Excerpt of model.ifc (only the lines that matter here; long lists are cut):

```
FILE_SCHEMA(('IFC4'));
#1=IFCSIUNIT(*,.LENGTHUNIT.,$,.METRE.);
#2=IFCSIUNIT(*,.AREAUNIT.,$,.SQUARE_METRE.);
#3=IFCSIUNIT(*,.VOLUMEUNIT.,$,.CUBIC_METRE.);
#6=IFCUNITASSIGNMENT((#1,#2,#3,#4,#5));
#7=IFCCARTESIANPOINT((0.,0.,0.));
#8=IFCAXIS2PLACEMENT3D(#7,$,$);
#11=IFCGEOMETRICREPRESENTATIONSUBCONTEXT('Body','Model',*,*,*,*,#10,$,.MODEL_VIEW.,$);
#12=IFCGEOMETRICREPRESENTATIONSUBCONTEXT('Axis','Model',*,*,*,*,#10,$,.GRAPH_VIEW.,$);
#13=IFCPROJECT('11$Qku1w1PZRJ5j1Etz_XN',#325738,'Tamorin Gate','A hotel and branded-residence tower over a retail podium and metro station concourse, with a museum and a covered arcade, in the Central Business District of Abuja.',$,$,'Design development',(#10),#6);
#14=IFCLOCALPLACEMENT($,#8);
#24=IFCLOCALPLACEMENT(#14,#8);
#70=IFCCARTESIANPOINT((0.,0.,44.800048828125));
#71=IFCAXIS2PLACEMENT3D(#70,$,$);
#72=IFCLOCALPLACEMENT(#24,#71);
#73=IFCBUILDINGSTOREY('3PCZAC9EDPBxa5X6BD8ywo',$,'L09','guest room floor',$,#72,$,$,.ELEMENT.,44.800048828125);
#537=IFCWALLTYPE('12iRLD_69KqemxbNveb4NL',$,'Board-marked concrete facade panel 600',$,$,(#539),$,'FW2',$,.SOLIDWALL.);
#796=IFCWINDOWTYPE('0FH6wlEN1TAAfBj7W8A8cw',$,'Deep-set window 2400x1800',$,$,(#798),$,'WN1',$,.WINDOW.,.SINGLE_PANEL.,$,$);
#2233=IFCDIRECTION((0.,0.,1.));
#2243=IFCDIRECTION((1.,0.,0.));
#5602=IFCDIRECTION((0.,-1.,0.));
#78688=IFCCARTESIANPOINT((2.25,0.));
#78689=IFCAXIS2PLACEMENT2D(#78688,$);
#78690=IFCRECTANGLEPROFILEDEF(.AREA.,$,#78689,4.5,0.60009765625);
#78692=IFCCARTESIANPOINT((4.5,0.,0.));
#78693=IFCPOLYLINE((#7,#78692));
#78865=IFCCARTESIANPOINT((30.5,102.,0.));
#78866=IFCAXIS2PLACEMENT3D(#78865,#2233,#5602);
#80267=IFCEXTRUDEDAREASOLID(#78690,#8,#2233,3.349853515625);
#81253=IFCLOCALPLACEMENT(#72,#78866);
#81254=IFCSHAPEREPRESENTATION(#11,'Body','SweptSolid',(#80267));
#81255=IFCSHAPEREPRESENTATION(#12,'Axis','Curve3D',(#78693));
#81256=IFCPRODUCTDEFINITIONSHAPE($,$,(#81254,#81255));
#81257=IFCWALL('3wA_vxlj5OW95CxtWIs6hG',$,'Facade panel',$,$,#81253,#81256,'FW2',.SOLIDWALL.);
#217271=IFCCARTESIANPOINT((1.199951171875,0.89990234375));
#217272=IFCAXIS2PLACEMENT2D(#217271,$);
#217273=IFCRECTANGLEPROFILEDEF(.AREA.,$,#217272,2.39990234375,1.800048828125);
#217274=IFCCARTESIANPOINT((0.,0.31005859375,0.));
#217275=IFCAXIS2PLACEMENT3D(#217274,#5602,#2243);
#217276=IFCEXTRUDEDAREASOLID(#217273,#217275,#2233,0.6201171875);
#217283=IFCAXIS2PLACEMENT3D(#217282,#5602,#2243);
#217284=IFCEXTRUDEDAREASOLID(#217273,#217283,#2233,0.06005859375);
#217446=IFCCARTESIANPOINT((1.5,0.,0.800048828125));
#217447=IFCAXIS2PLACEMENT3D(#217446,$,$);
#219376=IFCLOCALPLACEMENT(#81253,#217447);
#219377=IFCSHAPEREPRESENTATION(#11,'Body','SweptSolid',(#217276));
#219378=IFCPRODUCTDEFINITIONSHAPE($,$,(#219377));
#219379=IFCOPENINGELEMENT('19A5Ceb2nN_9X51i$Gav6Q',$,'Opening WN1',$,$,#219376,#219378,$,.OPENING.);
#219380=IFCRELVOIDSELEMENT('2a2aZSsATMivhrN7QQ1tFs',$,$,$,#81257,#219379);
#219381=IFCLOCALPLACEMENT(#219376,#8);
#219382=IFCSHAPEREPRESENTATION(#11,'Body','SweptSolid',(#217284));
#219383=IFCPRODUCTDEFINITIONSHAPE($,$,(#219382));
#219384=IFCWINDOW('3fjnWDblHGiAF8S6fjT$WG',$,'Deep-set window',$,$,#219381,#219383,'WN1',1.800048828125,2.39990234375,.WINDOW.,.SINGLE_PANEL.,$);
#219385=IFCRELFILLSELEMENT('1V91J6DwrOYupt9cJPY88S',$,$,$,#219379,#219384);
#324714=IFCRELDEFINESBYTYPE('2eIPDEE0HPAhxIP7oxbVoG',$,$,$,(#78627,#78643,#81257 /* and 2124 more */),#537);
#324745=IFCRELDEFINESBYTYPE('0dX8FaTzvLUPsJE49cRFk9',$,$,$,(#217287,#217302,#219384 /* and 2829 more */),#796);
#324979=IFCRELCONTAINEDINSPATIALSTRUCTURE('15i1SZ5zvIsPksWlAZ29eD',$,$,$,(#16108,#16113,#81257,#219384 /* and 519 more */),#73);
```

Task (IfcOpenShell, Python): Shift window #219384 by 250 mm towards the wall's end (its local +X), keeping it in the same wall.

```python
import ifcopenshell
import ifcopenshell.api.geometry
import ifcopenshell.util.placement
import ifcopenshell.util.unit

model = ifcopenshell.open("model.ifc")
unit_scale = ifcopenshell.util.unit.calculate_unit_scale(model)

window = model.by_guid("3fjnWDblHGiAF8S6fjT$WG")
opening = window.FillsVoids[0].RelatingOpeningElement
wall = opening.VoidsElements[0].RelatingBuildingElement

wall_matrix = ifcopenshell.util.placement.get_local_placement(wall.ObjectPlacement)
shift = wall_matrix[:3, 0] * 0.25 / unit_scale
before = ifcopenshell.util.placement.get_local_placement(window.ObjectPlacement)[:3, 3].copy()

# The window is placed relative to its opening, so it follows when the opening moves.
matrix = ifcopenshell.util.placement.get_local_placement(opening.ObjectPlacement)
matrix[:3, 3] += shift
ifcopenshell.api.geometry.edit_object_placement(
    model, product=opening, matrix=matrix, is_si=False, should_transform_children=True
)

after = ifcopenshell.util.placement.get_local_placement(window.ObjectPlacement)[:3, 3]
print("window moved by", (after - before).round(3) + 0.0)

model.write("model_v2.ifc")
```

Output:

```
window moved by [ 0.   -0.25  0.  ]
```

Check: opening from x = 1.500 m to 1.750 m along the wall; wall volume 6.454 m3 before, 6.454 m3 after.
